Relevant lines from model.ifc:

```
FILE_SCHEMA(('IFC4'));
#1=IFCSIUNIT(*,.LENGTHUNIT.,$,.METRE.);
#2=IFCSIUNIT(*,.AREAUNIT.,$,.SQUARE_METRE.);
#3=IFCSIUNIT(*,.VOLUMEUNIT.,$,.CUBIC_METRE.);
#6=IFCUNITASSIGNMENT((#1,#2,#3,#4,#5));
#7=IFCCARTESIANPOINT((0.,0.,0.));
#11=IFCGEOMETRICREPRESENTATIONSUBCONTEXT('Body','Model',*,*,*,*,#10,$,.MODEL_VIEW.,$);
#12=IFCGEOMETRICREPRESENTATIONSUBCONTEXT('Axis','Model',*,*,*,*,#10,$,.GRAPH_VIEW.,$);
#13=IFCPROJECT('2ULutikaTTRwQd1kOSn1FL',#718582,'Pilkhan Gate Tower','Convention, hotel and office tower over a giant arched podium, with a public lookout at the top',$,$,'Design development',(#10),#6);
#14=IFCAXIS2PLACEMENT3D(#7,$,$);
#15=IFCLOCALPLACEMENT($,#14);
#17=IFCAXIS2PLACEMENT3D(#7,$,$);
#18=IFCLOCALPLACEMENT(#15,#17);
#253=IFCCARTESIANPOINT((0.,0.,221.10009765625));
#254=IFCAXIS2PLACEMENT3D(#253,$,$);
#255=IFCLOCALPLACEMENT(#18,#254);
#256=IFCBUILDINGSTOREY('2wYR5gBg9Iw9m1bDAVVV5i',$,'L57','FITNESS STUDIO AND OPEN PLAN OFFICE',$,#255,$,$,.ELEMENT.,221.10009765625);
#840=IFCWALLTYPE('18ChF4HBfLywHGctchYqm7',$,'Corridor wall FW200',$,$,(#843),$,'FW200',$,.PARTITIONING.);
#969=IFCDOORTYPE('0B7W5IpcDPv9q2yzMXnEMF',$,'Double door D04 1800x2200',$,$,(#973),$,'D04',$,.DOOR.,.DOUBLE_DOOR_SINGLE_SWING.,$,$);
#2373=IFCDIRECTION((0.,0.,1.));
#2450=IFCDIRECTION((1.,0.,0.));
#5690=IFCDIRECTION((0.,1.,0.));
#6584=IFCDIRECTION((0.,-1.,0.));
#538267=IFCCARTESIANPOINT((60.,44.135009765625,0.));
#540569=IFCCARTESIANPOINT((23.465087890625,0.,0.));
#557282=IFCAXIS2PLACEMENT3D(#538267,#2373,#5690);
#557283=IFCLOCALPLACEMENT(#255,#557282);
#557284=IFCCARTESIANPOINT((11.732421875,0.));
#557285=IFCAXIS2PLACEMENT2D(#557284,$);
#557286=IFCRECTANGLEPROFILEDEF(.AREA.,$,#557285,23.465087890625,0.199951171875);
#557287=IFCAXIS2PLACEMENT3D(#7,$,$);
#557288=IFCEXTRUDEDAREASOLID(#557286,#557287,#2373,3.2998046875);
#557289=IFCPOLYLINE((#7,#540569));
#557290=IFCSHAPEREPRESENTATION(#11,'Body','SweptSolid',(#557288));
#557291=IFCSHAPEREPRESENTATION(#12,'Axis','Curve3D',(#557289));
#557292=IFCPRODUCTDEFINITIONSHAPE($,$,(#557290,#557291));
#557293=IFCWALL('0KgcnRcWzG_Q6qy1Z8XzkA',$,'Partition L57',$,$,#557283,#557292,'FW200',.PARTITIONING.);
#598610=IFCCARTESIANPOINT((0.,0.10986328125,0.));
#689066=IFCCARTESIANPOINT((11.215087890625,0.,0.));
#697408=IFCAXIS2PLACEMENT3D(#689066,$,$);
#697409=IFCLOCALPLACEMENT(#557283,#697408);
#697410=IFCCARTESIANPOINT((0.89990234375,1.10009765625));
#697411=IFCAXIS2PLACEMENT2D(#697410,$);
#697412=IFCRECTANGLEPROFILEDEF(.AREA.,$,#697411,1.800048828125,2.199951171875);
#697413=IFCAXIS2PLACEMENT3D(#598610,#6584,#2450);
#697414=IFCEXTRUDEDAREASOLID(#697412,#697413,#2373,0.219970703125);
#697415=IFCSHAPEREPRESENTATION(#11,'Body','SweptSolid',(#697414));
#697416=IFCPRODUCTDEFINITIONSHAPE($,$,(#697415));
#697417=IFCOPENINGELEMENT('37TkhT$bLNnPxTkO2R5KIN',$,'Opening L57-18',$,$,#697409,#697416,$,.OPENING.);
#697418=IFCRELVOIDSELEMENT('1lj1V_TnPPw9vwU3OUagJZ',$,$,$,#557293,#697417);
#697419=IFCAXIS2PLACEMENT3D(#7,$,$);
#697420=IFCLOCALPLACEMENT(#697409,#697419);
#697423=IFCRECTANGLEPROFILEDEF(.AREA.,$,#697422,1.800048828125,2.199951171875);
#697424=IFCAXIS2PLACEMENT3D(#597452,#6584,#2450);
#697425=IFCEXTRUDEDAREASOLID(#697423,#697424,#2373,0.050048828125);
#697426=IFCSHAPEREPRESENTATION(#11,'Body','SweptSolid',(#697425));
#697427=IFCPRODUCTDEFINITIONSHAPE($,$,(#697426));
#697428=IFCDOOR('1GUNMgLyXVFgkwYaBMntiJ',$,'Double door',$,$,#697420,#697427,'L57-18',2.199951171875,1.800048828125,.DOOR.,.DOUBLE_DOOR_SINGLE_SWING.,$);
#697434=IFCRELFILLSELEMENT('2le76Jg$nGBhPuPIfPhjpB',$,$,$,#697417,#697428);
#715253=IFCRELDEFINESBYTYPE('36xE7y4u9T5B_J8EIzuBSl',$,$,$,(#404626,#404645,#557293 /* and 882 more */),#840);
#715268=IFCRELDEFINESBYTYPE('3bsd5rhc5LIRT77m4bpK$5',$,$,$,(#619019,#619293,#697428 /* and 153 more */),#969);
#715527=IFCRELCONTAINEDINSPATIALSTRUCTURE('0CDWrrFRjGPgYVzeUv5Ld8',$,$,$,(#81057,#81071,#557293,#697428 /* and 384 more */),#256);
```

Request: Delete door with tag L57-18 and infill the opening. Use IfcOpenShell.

```python
import ifcopenshell
import ifcopenshell.api.feature
import ifcopenshell.api.root
import ifcopenshell.geom
import ifcopenshell.util.shape

model = ifcopenshell.open("model.ifc")
settings = ifcopenshell.geom.settings()


def volume(element):
    """Net volume in cubic metres, openings subtracted."""
    shape = ifcopenshell.geom.create_shape(settings, element)
    return ifcopenshell.util.shape.get_volume(shape.geometry)


door = model.by_guid("1GUNMgLyXVFgkwYaBMntiJ")
opening = door.FillsVoids[0].RelatingOpeningElement
wall = opening.VoidsElements[0].RelatingBuildingElement
before = volume(wall)

ifcopenshell.api.root.remove_product(model, product=door)
ifcopenshell.api.feature.remove_feature(model, feature=opening)

after = volume(wall)

print(f"wall volume {before:.3f} -> {after:.3f} m3")

model.write("model_updated.ifc")
```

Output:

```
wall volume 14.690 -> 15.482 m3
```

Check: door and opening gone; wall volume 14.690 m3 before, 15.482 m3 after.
